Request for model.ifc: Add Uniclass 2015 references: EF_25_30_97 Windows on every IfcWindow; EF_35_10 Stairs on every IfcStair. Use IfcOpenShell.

First a look at what the model holds.

```python
import ifcopenshell

model = ifcopenshell.open("model.ifc")
print(model.schema)
print("classifications:", [c.Name for c in model.by_type("IfcClassification")])
for ifc_class in ("IfcDoor", "IfcRoof", "IfcStair", "IfcWall", "IfcWindow"):
    print(ifc_class, len(model.by_type(ifc_class)))
```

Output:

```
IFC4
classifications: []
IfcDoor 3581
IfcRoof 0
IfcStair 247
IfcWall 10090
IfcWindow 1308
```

```python
import ifcopenshell
import ifcopenshell.api.classification

model = ifcopenshell.open("model.ifc")

system = ifcopenshell.api.classification.add_classification(model, classification="Uniclass 2015")

codes = {
    "IfcWindow": ("EF_25_30_97", "Windows"),
    "IfcStair": ("EF_35_10", "Stairs"),
}
for ifc_class, (code, name) in codes.items():
    products = model.by_type(ifc_class)
    ifcopenshell.api.classification.add_reference(
        model, products=products, classification=system, identification=code, name=name
    )
    print(code, len(products))

model.write("model_edited.ifc")
```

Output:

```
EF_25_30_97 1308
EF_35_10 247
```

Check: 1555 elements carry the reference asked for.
